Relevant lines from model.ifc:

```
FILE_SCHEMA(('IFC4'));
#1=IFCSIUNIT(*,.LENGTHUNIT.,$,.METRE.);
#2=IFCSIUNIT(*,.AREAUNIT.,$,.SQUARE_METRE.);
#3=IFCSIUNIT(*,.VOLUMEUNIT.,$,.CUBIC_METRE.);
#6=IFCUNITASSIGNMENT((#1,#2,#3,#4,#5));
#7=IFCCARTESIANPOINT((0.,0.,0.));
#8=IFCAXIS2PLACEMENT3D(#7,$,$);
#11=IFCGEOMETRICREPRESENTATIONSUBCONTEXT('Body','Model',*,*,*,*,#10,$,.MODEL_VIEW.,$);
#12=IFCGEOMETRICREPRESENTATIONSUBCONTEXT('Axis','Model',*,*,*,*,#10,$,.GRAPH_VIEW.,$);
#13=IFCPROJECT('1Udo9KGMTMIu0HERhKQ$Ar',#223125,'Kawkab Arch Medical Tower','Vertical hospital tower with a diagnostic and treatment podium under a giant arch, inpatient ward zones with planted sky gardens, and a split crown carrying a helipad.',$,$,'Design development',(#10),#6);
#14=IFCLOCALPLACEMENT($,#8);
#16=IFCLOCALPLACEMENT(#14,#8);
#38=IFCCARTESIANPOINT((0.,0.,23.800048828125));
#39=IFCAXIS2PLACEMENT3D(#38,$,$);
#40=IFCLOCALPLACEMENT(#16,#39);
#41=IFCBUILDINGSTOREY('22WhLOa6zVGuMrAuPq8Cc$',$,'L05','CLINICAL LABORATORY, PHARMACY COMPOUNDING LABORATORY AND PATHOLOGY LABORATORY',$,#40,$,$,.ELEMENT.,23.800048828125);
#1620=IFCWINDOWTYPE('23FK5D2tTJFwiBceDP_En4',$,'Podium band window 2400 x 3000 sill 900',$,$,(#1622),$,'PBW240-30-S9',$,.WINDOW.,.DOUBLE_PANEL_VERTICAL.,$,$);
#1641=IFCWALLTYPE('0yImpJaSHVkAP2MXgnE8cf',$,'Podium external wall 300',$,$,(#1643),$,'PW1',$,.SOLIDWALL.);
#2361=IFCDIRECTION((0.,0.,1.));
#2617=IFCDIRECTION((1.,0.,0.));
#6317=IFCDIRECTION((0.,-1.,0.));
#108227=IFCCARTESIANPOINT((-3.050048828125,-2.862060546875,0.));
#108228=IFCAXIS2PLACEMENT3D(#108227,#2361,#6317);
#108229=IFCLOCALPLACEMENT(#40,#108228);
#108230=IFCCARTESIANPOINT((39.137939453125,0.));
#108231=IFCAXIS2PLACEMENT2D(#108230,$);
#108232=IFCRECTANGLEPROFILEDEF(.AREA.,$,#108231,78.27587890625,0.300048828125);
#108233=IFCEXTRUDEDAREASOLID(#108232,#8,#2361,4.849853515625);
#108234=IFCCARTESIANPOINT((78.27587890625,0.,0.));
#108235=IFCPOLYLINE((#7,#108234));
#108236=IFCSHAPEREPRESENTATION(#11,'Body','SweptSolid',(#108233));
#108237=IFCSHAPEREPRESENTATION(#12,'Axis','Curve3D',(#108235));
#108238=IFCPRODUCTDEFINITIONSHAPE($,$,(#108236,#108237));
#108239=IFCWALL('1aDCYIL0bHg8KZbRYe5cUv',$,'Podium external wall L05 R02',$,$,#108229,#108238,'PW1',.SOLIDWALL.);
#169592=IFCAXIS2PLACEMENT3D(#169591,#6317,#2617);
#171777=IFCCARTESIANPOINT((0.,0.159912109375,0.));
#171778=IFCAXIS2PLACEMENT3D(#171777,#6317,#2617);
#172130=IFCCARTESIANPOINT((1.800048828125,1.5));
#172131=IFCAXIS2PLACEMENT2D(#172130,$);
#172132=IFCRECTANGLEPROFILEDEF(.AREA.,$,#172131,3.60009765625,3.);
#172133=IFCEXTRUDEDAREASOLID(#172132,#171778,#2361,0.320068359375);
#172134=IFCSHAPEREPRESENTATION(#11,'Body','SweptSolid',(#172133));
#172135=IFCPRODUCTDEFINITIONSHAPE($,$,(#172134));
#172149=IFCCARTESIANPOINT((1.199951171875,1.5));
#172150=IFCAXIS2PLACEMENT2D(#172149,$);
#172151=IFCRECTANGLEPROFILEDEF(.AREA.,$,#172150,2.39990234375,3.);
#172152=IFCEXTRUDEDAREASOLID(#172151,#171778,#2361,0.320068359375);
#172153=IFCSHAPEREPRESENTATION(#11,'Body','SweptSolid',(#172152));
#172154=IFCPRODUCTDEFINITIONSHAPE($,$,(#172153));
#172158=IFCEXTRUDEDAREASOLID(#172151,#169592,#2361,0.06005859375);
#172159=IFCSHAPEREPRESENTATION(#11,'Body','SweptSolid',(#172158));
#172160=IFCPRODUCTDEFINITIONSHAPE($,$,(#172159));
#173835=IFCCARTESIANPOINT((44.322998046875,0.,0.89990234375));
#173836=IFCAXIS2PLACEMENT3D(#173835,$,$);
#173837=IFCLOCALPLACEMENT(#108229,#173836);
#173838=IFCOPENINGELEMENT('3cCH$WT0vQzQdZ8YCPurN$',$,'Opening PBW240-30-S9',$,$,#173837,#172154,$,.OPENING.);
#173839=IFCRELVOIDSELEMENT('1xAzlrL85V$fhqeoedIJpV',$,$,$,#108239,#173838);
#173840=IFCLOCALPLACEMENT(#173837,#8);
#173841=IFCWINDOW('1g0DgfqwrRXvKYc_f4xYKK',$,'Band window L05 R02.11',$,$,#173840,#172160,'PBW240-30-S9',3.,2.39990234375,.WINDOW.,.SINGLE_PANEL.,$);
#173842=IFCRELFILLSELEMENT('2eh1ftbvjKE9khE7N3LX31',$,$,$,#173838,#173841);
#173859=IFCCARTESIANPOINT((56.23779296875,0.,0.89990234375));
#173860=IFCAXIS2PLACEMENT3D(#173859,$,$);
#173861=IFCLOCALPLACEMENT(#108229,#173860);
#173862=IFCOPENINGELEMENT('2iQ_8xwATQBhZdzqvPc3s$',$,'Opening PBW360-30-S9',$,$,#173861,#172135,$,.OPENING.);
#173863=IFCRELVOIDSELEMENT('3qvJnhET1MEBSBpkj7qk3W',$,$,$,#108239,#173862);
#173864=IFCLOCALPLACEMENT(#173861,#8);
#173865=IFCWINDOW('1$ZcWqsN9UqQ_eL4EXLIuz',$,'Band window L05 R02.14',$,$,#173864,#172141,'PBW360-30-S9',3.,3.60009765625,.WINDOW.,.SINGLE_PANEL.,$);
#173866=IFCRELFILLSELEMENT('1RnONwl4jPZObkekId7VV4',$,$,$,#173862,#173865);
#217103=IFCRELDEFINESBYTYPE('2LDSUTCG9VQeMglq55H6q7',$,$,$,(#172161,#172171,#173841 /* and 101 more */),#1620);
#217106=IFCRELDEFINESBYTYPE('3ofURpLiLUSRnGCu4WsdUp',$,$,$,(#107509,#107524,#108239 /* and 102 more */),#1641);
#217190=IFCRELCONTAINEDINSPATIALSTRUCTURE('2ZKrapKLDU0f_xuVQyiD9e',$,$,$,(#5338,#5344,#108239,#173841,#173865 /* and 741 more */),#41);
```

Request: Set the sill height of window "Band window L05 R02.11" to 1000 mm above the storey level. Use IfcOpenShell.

```python
import numpy as np
import ifcopenshell
import ifcopenshell.api.geometry
import ifcopenshell.geom
import ifcopenshell.util.element
import ifcopenshell.util.placement
import ifcopenshell.util.shape
import ifcopenshell.util.unit

model = ifcopenshell.open("model.ifc")
unit_scale = ifcopenshell.util.unit.calculate_unit_scale(model)

window = model.by_guid("1g0DgfqwrRXvKYc_f4xYKK")
opening = window.FillsVoids[0].RelatingOpeningElement
storey = ifcopenshell.util.element.get_container(window, ifc_class="IfcBuildingStorey")
level = ifcopenshell.util.placement.get_local_placement(storey.ObjectPlacement)[2, 3]

# The opening's origin need not be at the sill, so measure its lowest point.
shape = ifcopenshell.geom.create_shape(ifcopenshell.geom.settings(), opening)
bottom = ifcopenshell.util.shape.get_shape_bottom_elevation(shape, shape.geometry) / unit_scale
dz = level + 1 / unit_scale - bottom

shift = np.array([0.0, 0.0, dz])
# The window is placed relative to its opening, so it follows when the opening moves.
matrix = ifcopenshell.util.placement.get_local_placement(opening.ObjectPlacement)
matrix[:3, 3] += shift
ifcopenshell.api.geometry.edit_object_placement(
    model, product=opening, matrix=matrix, is_si=False, should_transform_children=True
)

print(f"moved by {dz * unit_scale:+.3f} m")

model.write("model_updated.ifc")
```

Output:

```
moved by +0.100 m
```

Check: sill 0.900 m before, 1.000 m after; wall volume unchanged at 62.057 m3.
